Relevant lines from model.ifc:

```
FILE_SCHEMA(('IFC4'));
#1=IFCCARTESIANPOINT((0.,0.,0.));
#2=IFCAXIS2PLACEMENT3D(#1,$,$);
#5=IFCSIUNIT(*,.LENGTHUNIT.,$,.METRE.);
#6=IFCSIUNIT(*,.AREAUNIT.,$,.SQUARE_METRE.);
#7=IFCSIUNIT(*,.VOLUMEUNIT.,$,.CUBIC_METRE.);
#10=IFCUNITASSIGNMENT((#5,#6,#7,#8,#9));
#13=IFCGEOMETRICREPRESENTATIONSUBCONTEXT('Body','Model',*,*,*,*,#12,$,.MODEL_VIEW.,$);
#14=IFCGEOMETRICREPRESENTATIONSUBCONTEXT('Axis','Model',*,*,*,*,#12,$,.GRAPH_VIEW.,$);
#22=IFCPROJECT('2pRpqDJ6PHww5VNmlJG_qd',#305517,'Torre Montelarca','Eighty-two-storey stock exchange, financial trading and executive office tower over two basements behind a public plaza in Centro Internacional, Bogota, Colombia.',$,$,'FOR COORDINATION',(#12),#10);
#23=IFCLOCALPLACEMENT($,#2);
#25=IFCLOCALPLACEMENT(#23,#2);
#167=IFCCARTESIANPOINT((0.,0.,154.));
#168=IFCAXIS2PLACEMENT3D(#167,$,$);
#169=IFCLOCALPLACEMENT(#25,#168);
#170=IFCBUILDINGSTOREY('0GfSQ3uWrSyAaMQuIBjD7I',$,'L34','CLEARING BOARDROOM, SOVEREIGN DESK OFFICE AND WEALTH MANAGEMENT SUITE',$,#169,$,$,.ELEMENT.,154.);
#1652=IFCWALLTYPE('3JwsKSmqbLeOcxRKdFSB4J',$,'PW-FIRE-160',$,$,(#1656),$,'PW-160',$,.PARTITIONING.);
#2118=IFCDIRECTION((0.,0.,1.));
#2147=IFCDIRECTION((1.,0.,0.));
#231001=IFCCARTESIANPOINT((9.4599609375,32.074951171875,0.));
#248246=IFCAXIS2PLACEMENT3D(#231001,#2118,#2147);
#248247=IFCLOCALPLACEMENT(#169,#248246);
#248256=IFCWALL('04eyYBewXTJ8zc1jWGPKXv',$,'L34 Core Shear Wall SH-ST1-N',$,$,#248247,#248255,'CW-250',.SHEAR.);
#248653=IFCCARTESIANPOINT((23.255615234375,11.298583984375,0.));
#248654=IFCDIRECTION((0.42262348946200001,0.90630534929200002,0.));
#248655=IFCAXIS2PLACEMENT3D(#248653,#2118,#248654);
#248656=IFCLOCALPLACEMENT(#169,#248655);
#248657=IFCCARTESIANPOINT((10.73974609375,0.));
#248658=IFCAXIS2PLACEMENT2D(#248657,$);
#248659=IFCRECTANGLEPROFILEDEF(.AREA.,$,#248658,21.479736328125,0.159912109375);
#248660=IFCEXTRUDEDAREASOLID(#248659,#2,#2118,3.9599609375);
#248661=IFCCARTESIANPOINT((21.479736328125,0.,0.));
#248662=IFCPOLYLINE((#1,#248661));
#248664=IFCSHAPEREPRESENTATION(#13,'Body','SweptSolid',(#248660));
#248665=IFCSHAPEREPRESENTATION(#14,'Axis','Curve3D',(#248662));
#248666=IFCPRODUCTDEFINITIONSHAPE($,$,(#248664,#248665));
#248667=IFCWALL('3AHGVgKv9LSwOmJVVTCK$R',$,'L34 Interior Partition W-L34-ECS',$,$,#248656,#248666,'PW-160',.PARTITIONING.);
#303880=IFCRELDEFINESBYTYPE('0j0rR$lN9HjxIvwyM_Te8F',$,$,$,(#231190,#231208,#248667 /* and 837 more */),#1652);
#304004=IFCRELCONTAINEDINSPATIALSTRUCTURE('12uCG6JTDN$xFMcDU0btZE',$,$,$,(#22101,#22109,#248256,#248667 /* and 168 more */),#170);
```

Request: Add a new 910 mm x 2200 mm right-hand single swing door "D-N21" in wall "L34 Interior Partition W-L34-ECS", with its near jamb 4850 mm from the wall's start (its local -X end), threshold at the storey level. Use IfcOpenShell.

```python
import numpy as np
import ifcopenshell
import ifcopenshell.api.feature
import ifcopenshell.api.geometry
import ifcopenshell.api.root
import ifcopenshell.api.spatial
import ifcopenshell.geom
import ifcopenshell.util.element
import ifcopenshell.util.placement
import ifcopenshell.util.representation
import ifcopenshell.util.shape
import ifcopenshell.util.unit

model = ifcopenshell.open("model.ifc")
unit_scale = ifcopenshell.util.unit.calculate_unit_scale(model)
settings = ifcopenshell.geom.settings()


def volume(element):
    """Net volume in cubic metres, openings subtracted."""
    shape = ifcopenshell.geom.create_shape(settings, element)
    return ifcopenshell.util.shape.get_volume(shape.geometry)


wall = model.by_guid("3AHGVgKv9LSwOmJVVTCK$R")
storey = ifcopenshell.util.element.get_container(wall, ifc_class="IfcBuildingStorey")
context = ifcopenshell.util.representation.get_context(model, "Model", "Body", "MODEL_VIEW")
before = volume(wall)

width, height, from_end, sill = 0.91, 2.2, 4.85, 0.0  # metres

# The wall runs along its own X axis, and the end named is its -X end.
wall_shape = ifcopenshell.geom.create_shape(settings, wall)
x, y, z = ifcopenshell.util.shape.get_vertices(wall_shape.geometry).T
start = x.min() + from_end
face, thickness = float(y.min()), float(y.max() - y.min())
wall_matrix = ifcopenshell.util.placement.get_local_placement(wall.ObjectPlacement)
level = ifcopenshell.util.placement.get_local_placement(storey.ObjectPlacement)[2, 3]


def in_wall(x, y):
    """Placement at x, y metres in the wall's axes, at sill height."""
    matrix = wall_matrix.copy()
    matrix[:, 3] = wall_matrix @ np.array([x / unit_scale, y / unit_scale, 0.0, 1.0])
    matrix[2, 3] = level + sill / unit_scale
    return matrix


# Opening: a box that overshoots both wall faces by 50 mm.
opening = ifcopenshell.api.root.create_entity(model, ifc_class="IfcOpeningElement", predefined_type="OPENING")
box = ifcopenshell.api.geometry.add_wall_representation(
    model, context=context, length=width, height=height, thickness=thickness + 0.1
)
ifcopenshell.api.geometry.assign_representation(model, product=opening, representation=box)
ifcopenshell.api.geometry.edit_object_placement(model, product=opening, matrix=in_wall(start, face - 0.05), is_si=False)
ifcopenshell.api.feature.add_feature(model, feature=opening, element=wall)

door = ifcopenshell.api.root.create_entity(model, ifc_class="IfcDoor", name="D-N21", predefined_type="DOOR")
door.OverallWidth, door.OverallHeight = width / unit_scale, height / unit_scale
door.OperationType = "SINGLE_SWING_RIGHT"
body = ifcopenshell.api.geometry.add_door_representation(
    model,
    context=context,
    overall_width=door.OverallWidth,
    overall_height=door.OverallHeight,
    operation_type="SINGLE_SWING_RIGHT",
    lining_properties={"LiningDepth": thickness / unit_scale, "ThresholdDepth": thickness / unit_scale},
)
ifcopenshell.api.geometry.assign_representation(model, product=door, representation=body)
ifcopenshell.api.spatial.assign_container(model, products=[door], relating_structure=storey)
ifcopenshell.api.feature.add_filling(model, opening=opening, element=door)

# The lining spans the wall, so the door starts at the wall face.
ifcopenshell.api.geometry.edit_object_placement(model, product=door, matrix=in_wall(start, face), is_si=False)

after = volume(wall)

print(f"wall volume {before:.3f} -> {after:.3f} m3")

model.write("model_edited.ifc")
```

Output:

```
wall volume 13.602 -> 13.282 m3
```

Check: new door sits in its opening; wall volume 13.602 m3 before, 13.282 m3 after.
